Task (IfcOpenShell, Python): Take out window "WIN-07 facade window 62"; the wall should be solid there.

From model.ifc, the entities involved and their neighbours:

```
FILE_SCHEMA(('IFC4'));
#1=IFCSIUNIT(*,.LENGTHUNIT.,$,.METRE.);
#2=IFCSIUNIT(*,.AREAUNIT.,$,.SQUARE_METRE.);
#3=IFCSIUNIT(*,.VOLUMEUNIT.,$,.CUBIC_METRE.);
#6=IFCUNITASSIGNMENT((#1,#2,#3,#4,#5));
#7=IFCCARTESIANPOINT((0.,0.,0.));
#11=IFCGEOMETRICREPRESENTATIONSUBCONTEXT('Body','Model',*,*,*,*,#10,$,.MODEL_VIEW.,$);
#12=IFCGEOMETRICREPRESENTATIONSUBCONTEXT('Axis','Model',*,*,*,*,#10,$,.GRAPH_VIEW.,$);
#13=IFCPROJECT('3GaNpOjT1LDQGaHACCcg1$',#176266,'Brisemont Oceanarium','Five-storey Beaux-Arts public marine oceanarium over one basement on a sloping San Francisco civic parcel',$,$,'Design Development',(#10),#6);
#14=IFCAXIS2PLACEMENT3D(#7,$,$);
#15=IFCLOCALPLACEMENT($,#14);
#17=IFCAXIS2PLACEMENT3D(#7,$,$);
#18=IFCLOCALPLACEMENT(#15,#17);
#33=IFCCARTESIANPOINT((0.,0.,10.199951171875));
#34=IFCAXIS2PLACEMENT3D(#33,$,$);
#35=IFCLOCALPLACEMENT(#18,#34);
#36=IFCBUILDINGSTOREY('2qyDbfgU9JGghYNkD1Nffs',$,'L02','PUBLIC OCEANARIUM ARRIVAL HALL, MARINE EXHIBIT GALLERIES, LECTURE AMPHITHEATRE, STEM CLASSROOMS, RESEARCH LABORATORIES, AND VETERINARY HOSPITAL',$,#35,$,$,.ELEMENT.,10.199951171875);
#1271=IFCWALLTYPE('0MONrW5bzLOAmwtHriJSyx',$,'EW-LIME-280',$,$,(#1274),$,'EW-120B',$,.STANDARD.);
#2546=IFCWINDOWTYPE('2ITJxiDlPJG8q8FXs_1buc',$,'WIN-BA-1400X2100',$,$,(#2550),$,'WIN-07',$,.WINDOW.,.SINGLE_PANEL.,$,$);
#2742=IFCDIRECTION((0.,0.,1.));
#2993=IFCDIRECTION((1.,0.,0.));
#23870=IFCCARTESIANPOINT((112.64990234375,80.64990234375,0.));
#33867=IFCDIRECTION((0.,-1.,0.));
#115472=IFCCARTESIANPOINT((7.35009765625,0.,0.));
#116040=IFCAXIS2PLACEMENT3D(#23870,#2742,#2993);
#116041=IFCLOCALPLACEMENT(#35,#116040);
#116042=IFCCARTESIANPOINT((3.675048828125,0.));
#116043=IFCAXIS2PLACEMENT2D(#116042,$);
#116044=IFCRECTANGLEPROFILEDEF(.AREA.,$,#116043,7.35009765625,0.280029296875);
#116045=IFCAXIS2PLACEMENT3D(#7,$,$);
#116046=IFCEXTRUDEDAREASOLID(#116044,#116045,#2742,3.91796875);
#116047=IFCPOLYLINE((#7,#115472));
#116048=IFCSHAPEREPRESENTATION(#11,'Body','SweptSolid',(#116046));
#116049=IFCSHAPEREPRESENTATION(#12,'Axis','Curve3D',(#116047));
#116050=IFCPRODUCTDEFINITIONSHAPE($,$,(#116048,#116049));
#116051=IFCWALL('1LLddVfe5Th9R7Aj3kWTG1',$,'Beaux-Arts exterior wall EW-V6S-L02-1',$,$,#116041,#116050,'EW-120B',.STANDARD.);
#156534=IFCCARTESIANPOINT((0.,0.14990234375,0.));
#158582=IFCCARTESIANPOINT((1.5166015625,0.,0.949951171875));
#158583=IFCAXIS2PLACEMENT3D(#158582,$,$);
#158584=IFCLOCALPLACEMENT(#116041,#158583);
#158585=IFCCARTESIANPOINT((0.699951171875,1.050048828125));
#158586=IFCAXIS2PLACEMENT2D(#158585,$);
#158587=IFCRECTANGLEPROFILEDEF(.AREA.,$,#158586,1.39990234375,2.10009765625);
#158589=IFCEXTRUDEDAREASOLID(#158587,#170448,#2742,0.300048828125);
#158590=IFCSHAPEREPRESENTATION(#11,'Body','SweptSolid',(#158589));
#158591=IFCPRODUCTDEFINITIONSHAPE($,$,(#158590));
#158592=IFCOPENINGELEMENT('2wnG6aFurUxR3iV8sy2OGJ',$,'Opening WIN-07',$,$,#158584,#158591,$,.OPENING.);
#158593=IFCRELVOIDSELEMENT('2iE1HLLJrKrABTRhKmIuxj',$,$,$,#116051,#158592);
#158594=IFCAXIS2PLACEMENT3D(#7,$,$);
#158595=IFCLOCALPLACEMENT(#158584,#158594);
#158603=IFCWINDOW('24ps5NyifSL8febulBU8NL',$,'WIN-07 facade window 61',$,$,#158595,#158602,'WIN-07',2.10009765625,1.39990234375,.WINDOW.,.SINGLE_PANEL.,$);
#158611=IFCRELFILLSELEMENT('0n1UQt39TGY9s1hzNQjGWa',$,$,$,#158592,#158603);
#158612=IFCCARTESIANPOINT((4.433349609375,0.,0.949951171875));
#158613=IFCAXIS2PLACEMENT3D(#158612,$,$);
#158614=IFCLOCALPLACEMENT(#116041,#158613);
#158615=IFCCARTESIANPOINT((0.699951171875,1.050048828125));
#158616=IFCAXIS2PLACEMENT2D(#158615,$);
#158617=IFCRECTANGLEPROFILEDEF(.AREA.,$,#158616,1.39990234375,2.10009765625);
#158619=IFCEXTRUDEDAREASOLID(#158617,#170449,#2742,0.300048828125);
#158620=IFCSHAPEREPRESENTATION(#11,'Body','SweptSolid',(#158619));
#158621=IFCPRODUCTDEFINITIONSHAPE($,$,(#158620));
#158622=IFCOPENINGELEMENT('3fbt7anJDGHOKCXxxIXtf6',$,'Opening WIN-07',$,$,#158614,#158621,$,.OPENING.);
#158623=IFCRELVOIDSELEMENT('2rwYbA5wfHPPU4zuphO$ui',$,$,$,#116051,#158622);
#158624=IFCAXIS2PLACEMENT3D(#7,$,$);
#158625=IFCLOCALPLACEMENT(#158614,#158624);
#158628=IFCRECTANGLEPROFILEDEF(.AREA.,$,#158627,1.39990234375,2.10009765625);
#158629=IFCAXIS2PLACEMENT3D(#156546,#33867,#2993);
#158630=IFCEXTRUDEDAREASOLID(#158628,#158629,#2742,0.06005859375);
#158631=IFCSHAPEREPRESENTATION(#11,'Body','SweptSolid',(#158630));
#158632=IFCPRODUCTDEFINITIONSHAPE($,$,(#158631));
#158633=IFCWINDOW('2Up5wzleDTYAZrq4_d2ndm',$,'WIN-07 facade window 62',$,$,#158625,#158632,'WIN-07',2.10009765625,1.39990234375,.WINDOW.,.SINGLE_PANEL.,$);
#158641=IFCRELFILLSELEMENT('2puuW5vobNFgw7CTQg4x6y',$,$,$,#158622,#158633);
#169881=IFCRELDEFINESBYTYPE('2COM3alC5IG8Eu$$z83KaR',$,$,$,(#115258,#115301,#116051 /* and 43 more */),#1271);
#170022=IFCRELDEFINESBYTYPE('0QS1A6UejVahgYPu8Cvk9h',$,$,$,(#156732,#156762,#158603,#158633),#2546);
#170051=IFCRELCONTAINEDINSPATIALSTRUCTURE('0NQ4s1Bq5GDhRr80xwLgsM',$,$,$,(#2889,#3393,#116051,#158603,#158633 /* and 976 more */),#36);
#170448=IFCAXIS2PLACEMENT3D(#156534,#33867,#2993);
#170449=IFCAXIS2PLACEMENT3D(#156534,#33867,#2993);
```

```python
import ifcopenshell
import ifcopenshell.api.feature
import ifcopenshell.api.root
import ifcopenshell.geom
import ifcopenshell.util.shape

model = ifcopenshell.open("model.ifc")
settings = ifcopenshell.geom.settings()


def volume(element):
    """Net volume in cubic metres, openings subtracted."""
    shape = ifcopenshell.geom.create_shape(settings, element)
    return ifcopenshell.util.shape.get_volume(shape.geometry)


window = model.by_id(158633)
opening = window.FillsVoids[0].RelatingOpeningElement
wall = opening.VoidsElements[0].RelatingBuildingElement
before = volume(wall)

ifcopenshell.api.root.remove_product(model, product=window)
ifcopenshell.api.feature.remove_feature(model, feature=opening)

after = volume(wall)

print(f"wall volume {before:.3f} -> {after:.3f} m3")

model.write("model_edited.ifc")
```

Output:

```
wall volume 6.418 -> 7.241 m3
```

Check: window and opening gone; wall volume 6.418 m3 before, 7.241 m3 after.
